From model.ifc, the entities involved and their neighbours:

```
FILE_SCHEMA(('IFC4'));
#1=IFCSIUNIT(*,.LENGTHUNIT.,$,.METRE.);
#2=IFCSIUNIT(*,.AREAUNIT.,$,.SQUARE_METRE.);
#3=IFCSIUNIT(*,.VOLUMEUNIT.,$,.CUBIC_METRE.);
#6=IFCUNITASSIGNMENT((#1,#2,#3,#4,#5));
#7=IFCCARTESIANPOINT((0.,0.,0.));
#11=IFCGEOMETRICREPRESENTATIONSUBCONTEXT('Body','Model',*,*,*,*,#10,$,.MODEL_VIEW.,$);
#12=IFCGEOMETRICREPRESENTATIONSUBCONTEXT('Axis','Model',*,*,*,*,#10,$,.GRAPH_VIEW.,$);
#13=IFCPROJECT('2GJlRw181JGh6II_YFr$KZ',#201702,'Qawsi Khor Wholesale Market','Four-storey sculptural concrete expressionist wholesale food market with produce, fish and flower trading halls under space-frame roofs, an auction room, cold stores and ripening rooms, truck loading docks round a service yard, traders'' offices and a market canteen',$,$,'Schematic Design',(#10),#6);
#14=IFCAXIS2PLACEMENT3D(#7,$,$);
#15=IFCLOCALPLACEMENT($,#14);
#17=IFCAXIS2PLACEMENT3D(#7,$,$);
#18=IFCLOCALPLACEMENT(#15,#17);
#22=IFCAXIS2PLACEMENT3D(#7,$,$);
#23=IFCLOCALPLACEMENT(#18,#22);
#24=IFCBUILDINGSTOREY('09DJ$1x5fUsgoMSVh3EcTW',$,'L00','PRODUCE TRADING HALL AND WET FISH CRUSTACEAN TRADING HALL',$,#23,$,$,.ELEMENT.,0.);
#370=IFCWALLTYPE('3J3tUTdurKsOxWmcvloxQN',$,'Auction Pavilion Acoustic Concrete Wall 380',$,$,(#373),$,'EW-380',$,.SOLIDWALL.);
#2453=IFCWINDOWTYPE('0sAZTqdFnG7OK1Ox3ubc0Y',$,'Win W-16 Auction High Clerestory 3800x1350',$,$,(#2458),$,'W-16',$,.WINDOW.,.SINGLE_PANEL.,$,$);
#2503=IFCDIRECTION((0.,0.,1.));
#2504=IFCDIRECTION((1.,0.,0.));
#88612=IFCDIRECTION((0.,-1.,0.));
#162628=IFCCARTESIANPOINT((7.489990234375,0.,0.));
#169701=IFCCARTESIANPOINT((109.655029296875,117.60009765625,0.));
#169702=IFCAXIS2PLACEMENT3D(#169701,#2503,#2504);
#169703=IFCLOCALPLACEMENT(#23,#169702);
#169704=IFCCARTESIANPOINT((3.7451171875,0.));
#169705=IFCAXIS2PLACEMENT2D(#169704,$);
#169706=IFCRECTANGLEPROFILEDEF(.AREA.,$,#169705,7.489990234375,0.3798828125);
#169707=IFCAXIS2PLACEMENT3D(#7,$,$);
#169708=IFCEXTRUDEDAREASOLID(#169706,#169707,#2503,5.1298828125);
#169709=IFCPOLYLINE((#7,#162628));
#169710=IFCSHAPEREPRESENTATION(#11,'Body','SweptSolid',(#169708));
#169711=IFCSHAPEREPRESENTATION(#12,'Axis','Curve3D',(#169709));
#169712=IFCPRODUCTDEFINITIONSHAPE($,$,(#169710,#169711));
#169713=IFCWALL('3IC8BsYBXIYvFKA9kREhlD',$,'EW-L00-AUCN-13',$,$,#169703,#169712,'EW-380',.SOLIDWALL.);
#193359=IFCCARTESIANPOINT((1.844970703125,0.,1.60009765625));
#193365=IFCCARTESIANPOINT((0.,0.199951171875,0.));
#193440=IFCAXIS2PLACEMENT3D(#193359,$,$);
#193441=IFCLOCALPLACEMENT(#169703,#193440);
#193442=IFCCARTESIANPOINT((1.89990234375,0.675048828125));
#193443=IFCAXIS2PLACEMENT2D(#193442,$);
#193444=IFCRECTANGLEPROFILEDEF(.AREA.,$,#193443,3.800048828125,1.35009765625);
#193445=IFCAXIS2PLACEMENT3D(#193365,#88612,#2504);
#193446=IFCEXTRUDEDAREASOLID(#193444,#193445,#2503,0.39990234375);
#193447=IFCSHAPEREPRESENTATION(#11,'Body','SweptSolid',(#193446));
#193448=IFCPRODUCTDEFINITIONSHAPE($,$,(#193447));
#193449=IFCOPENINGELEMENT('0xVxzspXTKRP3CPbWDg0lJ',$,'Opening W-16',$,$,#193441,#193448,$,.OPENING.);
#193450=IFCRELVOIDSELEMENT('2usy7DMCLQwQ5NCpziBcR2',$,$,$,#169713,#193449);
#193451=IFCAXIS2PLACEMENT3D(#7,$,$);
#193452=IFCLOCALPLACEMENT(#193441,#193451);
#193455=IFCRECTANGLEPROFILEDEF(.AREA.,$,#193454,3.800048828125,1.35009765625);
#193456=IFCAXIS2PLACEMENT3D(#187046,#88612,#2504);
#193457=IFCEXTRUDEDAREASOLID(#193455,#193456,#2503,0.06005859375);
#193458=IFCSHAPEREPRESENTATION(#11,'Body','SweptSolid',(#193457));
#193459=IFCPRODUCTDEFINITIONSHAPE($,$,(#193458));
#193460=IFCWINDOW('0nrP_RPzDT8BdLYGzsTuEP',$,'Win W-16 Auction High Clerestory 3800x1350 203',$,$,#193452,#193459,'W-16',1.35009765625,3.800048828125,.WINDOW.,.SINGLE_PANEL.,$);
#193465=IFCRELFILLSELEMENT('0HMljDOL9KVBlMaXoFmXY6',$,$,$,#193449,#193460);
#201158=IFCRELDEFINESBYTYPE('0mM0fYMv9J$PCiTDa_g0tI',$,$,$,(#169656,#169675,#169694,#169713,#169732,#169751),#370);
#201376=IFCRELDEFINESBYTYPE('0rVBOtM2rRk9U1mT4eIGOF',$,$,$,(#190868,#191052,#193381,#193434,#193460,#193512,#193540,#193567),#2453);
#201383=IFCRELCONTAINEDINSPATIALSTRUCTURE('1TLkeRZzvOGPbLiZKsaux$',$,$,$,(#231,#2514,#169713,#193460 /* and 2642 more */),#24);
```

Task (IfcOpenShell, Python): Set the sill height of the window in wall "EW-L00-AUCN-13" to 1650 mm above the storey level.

```python
import numpy as np
import ifcopenshell
import ifcopenshell.api.geometry
import ifcopenshell.geom
import ifcopenshell.util.element
import ifcopenshell.util.placement
import ifcopenshell.util.shape
import ifcopenshell.util.unit

model = ifcopenshell.open("model.ifc")
unit_scale = ifcopenshell.util.unit.calculate_unit_scale(model)

window = model.by_id(193460)
opening = window.FillsVoids[0].RelatingOpeningElement
storey = ifcopenshell.util.element.get_container(window, ifc_class="IfcBuildingStorey")
level = ifcopenshell.util.placement.get_local_placement(storey.ObjectPlacement)[2, 3]

# The opening's origin need not be at the sill, so measure its lowest point.
shape = ifcopenshell.geom.create_shape(ifcopenshell.geom.settings(), opening)
bottom = ifcopenshell.util.shape.get_shape_bottom_elevation(shape, shape.geometry) / unit_scale
dz = level + 1.65 - bottom

shift = np.array([0.0, 0.0, dz])
# The window is placed relative to its opening, so it follows when the opening moves.
matrix = ifcopenshell.util.placement.get_local_placement(opening.ObjectPlacement)
matrix[:3, 3] += shift
ifcopenshell.api.geometry.edit_object_placement(
    model, product=opening, matrix=matrix, is_si=False, should_transform_children=True
)

print(f"moved by {dz * unit_scale:+.3f} m")

model.write("model_updated.ifc")
```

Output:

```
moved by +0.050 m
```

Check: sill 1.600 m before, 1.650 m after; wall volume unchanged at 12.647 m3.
